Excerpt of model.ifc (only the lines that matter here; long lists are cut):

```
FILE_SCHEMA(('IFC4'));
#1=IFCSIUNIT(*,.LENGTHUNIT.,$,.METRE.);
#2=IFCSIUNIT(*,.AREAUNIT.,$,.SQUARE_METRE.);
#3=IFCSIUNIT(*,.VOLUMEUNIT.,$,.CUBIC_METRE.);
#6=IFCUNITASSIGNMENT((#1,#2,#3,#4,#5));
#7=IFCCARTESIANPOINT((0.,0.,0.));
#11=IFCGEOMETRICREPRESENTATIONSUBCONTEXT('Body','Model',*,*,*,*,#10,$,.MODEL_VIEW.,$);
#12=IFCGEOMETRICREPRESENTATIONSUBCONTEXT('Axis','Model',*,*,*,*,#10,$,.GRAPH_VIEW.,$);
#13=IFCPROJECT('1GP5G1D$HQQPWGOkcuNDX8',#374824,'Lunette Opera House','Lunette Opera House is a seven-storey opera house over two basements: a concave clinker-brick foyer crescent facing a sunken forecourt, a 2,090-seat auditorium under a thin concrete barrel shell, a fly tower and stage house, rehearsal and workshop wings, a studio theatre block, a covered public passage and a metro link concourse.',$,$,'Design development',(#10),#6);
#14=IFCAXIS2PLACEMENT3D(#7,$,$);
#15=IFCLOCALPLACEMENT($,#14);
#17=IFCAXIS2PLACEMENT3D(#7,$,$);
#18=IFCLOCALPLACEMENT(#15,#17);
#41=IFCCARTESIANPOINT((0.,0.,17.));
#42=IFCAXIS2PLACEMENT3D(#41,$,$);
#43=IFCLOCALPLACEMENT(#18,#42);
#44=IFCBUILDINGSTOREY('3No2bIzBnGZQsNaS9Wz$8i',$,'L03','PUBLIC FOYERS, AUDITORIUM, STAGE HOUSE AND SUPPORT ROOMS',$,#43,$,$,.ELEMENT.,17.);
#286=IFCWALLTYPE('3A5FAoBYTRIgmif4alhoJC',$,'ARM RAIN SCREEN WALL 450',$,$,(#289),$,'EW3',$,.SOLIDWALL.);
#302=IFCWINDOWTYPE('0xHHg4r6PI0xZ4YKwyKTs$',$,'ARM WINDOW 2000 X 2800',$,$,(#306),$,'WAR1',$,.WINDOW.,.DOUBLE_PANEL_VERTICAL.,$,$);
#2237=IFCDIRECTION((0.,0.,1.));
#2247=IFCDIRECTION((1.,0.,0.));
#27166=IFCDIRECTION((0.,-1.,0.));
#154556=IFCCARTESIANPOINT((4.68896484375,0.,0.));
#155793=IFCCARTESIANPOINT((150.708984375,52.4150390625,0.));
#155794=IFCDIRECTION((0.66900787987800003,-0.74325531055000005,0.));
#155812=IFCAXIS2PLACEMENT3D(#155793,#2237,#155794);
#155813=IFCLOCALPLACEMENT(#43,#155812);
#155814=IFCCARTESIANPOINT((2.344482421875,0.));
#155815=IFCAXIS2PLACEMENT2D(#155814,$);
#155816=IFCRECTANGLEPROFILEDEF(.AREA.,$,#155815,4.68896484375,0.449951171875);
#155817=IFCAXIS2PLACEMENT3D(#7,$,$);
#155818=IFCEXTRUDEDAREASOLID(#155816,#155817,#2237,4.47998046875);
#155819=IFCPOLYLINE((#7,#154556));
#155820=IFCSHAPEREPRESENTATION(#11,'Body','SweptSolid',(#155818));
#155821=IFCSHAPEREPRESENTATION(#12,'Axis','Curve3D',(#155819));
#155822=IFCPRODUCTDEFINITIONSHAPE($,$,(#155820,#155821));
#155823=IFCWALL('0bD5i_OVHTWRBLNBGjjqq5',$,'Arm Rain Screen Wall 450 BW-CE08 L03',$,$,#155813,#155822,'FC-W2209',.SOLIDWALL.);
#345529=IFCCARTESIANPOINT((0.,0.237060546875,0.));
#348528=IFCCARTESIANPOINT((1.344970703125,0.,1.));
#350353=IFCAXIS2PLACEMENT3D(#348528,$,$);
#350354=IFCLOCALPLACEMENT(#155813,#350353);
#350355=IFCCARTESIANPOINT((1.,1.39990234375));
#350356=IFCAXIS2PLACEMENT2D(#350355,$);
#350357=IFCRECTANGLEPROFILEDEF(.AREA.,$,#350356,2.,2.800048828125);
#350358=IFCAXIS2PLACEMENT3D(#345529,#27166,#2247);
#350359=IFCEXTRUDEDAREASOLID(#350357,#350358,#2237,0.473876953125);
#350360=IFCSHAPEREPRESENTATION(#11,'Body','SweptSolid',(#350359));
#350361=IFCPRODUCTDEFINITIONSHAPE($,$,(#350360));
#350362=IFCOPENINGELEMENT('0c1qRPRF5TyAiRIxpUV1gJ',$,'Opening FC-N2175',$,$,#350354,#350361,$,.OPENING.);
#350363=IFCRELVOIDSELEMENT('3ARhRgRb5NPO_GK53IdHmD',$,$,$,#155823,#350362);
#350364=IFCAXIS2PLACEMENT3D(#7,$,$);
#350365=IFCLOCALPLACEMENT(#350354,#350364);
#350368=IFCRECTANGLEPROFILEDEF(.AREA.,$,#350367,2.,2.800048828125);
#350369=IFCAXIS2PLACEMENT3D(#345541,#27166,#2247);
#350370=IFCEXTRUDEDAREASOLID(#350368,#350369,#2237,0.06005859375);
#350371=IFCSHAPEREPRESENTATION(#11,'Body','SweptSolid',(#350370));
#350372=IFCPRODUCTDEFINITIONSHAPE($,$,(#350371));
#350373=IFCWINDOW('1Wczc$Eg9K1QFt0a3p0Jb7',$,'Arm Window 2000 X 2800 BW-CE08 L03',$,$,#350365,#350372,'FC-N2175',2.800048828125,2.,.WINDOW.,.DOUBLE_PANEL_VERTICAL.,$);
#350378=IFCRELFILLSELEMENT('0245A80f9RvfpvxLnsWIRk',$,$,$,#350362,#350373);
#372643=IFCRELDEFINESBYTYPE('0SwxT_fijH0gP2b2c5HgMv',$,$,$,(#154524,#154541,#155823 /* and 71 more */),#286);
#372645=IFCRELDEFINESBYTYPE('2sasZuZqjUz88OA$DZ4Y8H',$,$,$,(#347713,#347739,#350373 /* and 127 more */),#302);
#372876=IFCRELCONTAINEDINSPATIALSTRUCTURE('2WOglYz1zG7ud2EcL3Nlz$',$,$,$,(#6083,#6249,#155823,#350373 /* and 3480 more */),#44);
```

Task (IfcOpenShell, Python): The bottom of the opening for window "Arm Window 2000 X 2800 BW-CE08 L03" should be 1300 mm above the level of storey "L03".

```python
import numpy as np
import ifcopenshell
import ifcopenshell.api.geometry
import ifcopenshell.geom
import ifcopenshell.util.element
import ifcopenshell.util.placement
import ifcopenshell.util.shape
import ifcopenshell.util.unit

model = ifcopenshell.open("model.ifc")
unit_scale = ifcopenshell.util.unit.calculate_unit_scale(model)

window = model.by_id(350373)
opening = window.FillsVoids[0].RelatingOpeningElement
storey = ifcopenshell.util.element.get_container(window, ifc_class="IfcBuildingStorey")
level = ifcopenshell.util.placement.get_local_placement(storey.ObjectPlacement)[2, 3]

# The opening's origin need not be at the sill, so measure its lowest point.
shape = ifcopenshell.geom.create_shape(ifcopenshell.geom.settings(), opening)
bottom = ifcopenshell.util.shape.get_shape_bottom_elevation(shape, shape.geometry) / unit_scale
dz = level + 1.3 - bottom

shift = np.array([0.0, 0.0, dz])
# The window is placed relative to its opening, so it follows when the opening moves.
matrix = ifcopenshell.util.placement.get_local_placement(opening.ObjectPlacement)
matrix[:3, 3] += shift
ifcopenshell.api.geometry.edit_object_placement(
    model, product=opening, matrix=matrix, is_si=False, should_transform_children=True
)

print(f"moved by {dz * unit_scale:+.3f} m")

model.write("model_v2.ifc")
```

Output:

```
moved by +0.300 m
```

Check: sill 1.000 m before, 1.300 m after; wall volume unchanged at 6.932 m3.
